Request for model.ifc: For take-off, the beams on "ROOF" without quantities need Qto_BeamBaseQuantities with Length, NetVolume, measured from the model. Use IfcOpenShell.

First a look at what the model holds.

```python
import ifcopenshell
import ifcopenshell.util.element
import ifcopenshell.util.unit

model = ifcopenshell.open("model.ifc")
print(model.schema)
for unit_type in ("LENGTHUNIT", "AREAUNIT", "VOLUMEUNIT"):
    print(unit_type, ifcopenshell.util.unit.calculate_unit_scale(model, unit_type))
storey = next(s for s in model.by_type("IfcBuildingStorey") if s.Name == "ROOF")
beams = [e for e in ifcopenshell.util.element.get_decomposition(storey) if e.is_a("IfcBeam")]
for e in sorted(beams, key=lambda e: e.id()):
    print(e.id(), e.is_a(), e.Name, list(ifcopenshell.util.element.get_psets(e, qtos_only=True)), sep=" | ")
```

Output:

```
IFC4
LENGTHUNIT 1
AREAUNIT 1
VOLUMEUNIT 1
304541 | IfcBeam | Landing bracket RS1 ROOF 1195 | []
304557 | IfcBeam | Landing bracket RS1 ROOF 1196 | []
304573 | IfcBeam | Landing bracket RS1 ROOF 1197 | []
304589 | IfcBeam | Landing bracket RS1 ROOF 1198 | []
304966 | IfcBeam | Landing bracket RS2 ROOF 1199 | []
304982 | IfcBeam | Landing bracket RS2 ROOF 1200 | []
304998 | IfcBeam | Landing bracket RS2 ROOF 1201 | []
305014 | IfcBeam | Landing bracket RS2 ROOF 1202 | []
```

```python
import ifcopenshell
import ifcopenshell.api.pset
import ifcopenshell.geom
import ifcopenshell.util.element
import ifcopenshell.util.shape
import ifcopenshell.util.unit

model = ifcopenshell.open("model.ifc")
unit_scale = ifcopenshell.util.unit.calculate_unit_scale(model)
volume_scale = ifcopenshell.util.unit.calculate_unit_scale(model, "VOLUMEUNIT")
settings = ifcopenshell.geom.settings()

storey = next(s for s in model.by_type("IfcBuildingStorey") if s.Name == "ROOF")
beams = [e for e in ifcopenshell.util.element.get_decomposition(storey) if e.is_a("IfcBeam")]

for e in sorted(beams, key=lambda e: e.id()):
    if ifcopenshell.util.element.get_psets(e, qtos_only=True, should_inherit=False):
        continue
    # Geometry comes back in metres, in the element's own axes.
    shape = ifcopenshell.geom.create_shape(settings, e)
    values = {
        "Length": ifcopenshell.util.shape.get_max_xyz(shape.geometry) / unit_scale,
        "NetVolume": ifcopenshell.util.shape.get_volume(shape.geometry) / volume_scale,
    }
    qto = ifcopenshell.api.pset.add_qto(model, product=e, name="Qto_BeamBaseQuantities")
    ifcopenshell.api.pset.edit_qto(model, qto=qto, properties=values)
    print(e.id(), {k: round(v, 3) for k, v in values.items()})

model.write("model_rev.ifc")
```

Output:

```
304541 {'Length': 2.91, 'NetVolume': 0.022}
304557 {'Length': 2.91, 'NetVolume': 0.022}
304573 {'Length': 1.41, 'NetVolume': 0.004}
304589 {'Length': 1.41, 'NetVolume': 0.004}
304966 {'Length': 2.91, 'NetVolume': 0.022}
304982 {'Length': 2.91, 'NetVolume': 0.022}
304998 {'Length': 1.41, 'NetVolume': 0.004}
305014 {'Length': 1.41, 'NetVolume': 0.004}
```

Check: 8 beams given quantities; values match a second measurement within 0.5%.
